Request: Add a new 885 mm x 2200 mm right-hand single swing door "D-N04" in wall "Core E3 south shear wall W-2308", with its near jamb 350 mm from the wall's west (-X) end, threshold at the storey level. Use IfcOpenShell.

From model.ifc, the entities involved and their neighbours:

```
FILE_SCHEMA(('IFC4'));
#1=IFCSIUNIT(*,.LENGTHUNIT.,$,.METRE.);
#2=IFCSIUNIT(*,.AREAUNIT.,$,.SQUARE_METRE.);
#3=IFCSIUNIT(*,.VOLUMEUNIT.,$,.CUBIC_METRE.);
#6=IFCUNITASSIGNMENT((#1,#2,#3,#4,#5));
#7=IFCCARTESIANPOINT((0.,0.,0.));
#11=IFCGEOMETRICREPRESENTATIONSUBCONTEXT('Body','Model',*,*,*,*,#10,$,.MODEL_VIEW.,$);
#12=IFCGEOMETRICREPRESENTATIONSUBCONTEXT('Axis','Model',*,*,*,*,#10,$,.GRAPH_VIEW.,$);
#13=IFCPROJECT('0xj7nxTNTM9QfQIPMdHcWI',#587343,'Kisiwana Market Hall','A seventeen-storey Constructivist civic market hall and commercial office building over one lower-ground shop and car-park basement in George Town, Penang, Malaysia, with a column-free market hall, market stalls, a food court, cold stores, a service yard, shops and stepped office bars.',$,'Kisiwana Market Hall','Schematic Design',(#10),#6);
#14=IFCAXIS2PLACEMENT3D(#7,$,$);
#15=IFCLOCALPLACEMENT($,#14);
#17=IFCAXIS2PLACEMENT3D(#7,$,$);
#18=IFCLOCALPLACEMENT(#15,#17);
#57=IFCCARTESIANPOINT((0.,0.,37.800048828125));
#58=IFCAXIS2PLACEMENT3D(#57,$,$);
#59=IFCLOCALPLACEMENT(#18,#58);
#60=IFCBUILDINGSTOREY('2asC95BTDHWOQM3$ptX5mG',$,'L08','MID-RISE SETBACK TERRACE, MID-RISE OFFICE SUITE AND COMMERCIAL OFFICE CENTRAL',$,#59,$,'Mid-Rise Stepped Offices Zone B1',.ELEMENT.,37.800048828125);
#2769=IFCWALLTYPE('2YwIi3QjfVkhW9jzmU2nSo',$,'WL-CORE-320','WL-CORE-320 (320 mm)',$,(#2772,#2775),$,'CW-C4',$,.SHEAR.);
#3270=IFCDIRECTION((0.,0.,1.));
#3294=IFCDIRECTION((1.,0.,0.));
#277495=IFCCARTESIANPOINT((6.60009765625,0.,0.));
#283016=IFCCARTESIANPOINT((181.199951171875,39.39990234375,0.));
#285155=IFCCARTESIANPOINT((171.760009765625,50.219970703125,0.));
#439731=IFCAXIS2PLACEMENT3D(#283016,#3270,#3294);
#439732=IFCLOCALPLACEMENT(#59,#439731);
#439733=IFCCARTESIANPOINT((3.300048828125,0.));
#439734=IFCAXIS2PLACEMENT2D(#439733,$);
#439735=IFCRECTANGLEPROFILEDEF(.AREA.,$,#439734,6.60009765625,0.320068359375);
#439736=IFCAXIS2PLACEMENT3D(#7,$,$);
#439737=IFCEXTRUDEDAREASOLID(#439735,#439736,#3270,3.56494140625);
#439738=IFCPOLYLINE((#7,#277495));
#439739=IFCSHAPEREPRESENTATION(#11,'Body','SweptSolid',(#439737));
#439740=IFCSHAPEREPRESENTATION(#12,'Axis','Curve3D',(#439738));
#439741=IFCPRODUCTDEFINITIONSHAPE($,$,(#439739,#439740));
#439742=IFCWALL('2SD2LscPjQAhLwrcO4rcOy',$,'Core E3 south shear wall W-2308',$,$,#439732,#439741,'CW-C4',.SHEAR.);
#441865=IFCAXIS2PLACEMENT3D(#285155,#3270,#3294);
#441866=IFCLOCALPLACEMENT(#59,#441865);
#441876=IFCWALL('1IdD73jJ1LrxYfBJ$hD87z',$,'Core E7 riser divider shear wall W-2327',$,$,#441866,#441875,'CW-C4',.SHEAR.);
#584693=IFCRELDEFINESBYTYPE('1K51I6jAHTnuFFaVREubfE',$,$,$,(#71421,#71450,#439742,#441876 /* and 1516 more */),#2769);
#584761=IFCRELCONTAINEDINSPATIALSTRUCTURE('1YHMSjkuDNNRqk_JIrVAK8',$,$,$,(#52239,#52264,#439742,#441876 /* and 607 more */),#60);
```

```python
import numpy as np
import ifcopenshell
import ifcopenshell.api.feature
import ifcopenshell.api.geometry
import ifcopenshell.api.root
import ifcopenshell.api.spatial
import ifcopenshell.geom
import ifcopenshell.util.element
import ifcopenshell.util.placement
import ifcopenshell.util.representation
import ifcopenshell.util.shape
import ifcopenshell.util.unit

model = ifcopenshell.open("model.ifc")
unit_scale = ifcopenshell.util.unit.calculate_unit_scale(model)
settings = ifcopenshell.geom.settings()


def volume(element):
    """Net volume in cubic metres, openings subtracted."""
    shape = ifcopenshell.geom.create_shape(settings, element)
    return ifcopenshell.util.shape.get_volume(shape.geometry)


wall = model.by_id(439742)
storey = ifcopenshell.util.element.get_container(wall, ifc_class="IfcBuildingStorey")
context = ifcopenshell.util.representation.get_context(model, "Model", "Body", "MODEL_VIEW")
before = volume(wall)

width, height, from_end, sill = 0.885, 2.2, 0.35, 0.0  # metres

# The wall runs along its own X axis, and the end named is its -X end.
wall_shape = ifcopenshell.geom.create_shape(settings, wall)
x, y, z = ifcopenshell.util.shape.get_vertices(wall_shape.geometry).T
start = x.min() + from_end
face, thickness = float(y.min()), float(y.max() - y.min())
wall_matrix = ifcopenshell.util.placement.get_local_placement(wall.ObjectPlacement)
level = ifcopenshell.util.placement.get_local_placement(storey.ObjectPlacement)[2, 3]


def in_wall(x, y):
    """Placement at x, y metres in the wall's axes, at sill height."""
    matrix = wall_matrix.copy()
    matrix[:, 3] = wall_matrix @ np.array([x / unit_scale, y / unit_scale, 0.0, 1.0])
    matrix[2, 3] = level + sill / unit_scale
    return matrix


# Opening: a box that overshoots both wall faces by 50 mm.
opening = ifcopenshell.api.root.create_entity(model, ifc_class="IfcOpeningElement", predefined_type="OPENING")
box = ifcopenshell.api.geometry.add_wall_representation(
    model, context=context, length=width, height=height, thickness=thickness + 0.1
)
ifcopenshell.api.geometry.assign_representation(model, product=opening, representation=box)
ifcopenshell.api.geometry.edit_object_placement(model, product=opening, matrix=in_wall(start, face - 0.05), is_si=False)
ifcopenshell.api.feature.add_feature(model, feature=opening, element=wall)

door = ifcopenshell.api.root.create_entity(model, ifc_class="IfcDoor", name="D-N04", predefined_type="DOOR")
door.OverallWidth, door.OverallHeight = width / unit_scale, height / unit_scale
door.OperationType = "SINGLE_SWING_RIGHT"
body = ifcopenshell.api.geometry.add_door_representation(
    model,
    context=context,
    overall_width=door.OverallWidth,
    overall_height=door.OverallHeight,
    operation_type="SINGLE_SWING_RIGHT",
    lining_properties={"LiningDepth": thickness / unit_scale, "ThresholdDepth": thickness / unit_scale},
)
ifcopenshell.api.geometry.assign_representation(model, product=door, representation=body)
ifcopenshell.api.spatial.assign_container(model, products=[door], relating_structure=storey)
ifcopenshell.api.feature.add_filling(model, opening=opening, element=door)

# The lining spans the wall, so the door starts at the wall face.
ifcopenshell.api.geometry.edit_object_placement(model, product=door, matrix=in_wall(start, face), is_si=False)

after = volume(wall)

print(f"wall volume {before:.3f} -> {after:.3f} m3")

model.write("model_updated.ifc")
```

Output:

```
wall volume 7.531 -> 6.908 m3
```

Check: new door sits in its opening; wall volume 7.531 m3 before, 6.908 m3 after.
